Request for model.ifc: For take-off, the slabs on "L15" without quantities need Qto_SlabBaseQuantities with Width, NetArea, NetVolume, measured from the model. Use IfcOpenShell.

First a look at what the model holds.

```python
import ifcopenshell
import ifcopenshell.util.element
import ifcopenshell.util.unit

model = ifcopenshell.open("model.ifc")
print(model.schema)
for unit_type in ("LENGTHUNIT", "AREAUNIT", "VOLUMEUNIT"):
    print(unit_type, ifcopenshell.util.unit.calculate_unit_scale(model, unit_type))
storey = next(s for s in model.by_type("IfcBuildingStorey") if s.Name == "L15")
slabs = [e for e in ifcopenshell.util.element.get_decomposition(storey) if e.is_a("IfcSlab")]
for e in sorted(slabs, key=lambda e: e.id()):
    print(e.id(), e.is_a(), e.Name, list(ifcopenshell.util.element.get_psets(e, qtos_only=True)), sep=" | ")
```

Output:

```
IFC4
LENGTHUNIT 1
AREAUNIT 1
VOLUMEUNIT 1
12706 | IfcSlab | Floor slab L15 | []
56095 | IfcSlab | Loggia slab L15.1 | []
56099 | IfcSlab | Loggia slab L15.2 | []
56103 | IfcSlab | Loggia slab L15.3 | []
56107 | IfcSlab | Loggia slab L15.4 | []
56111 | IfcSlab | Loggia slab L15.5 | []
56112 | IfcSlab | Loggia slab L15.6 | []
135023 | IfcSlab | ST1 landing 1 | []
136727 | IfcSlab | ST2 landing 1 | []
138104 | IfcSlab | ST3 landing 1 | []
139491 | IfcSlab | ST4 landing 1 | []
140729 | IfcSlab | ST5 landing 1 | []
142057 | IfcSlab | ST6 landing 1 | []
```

```python
import ifcopenshell
import ifcopenshell.api.pset
import ifcopenshell.geom
import ifcopenshell.util.element
import ifcopenshell.util.shape
import ifcopenshell.util.unit

model = ifcopenshell.open("model.ifc")
unit_scale = ifcopenshell.util.unit.calculate_unit_scale(model)
area_scale = ifcopenshell.util.unit.calculate_unit_scale(model, "AREAUNIT")
volume_scale = ifcopenshell.util.unit.calculate_unit_scale(model, "VOLUMEUNIT")
settings = ifcopenshell.geom.settings()

storey = next(s for s in model.by_type("IfcBuildingStorey") if s.Name == "L15")
slabs = [e for e in ifcopenshell.util.element.get_decomposition(storey) if e.is_a("IfcSlab")]

for e in sorted(slabs, key=lambda e: e.id()):
    if ifcopenshell.util.element.get_psets(e, qtos_only=True, should_inherit=False):
        continue
    # Geometry comes back in metres, in the element's own axes.
    shape = ifcopenshell.geom.create_shape(settings, e)
    values = {
        "Width": ifcopenshell.util.shape.get_z(shape.geometry) / unit_scale,
        "NetArea": ifcopenshell.util.shape.get_footprint_area(shape.geometry) / area_scale,
        "NetVolume": ifcopenshell.util.shape.get_volume(shape.geometry) / volume_scale,
    }
    qto = ifcopenshell.api.pset.add_qto(model, product=e, name="Qto_SlabBaseQuantities")
    ifcopenshell.api.pset.edit_qto(model, qto=qto, properties=values)
    print(e.id(), {k: round(v, 3) for k, v in values.items()})

model.write("model-out.ifc")
```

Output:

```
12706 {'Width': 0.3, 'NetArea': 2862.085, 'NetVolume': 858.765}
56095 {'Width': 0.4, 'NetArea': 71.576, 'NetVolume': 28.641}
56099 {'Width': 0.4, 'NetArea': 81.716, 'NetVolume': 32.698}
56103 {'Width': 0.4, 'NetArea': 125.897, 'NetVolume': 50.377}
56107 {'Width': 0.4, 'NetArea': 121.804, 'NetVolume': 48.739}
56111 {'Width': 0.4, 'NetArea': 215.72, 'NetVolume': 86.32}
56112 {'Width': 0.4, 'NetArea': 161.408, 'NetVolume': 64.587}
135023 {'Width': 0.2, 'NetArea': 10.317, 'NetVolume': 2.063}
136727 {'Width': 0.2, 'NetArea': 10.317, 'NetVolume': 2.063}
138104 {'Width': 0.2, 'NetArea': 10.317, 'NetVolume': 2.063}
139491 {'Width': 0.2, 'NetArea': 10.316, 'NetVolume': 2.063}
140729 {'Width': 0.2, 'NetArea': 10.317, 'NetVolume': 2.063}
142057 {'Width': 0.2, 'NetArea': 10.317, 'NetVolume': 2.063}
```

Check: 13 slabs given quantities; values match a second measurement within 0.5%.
